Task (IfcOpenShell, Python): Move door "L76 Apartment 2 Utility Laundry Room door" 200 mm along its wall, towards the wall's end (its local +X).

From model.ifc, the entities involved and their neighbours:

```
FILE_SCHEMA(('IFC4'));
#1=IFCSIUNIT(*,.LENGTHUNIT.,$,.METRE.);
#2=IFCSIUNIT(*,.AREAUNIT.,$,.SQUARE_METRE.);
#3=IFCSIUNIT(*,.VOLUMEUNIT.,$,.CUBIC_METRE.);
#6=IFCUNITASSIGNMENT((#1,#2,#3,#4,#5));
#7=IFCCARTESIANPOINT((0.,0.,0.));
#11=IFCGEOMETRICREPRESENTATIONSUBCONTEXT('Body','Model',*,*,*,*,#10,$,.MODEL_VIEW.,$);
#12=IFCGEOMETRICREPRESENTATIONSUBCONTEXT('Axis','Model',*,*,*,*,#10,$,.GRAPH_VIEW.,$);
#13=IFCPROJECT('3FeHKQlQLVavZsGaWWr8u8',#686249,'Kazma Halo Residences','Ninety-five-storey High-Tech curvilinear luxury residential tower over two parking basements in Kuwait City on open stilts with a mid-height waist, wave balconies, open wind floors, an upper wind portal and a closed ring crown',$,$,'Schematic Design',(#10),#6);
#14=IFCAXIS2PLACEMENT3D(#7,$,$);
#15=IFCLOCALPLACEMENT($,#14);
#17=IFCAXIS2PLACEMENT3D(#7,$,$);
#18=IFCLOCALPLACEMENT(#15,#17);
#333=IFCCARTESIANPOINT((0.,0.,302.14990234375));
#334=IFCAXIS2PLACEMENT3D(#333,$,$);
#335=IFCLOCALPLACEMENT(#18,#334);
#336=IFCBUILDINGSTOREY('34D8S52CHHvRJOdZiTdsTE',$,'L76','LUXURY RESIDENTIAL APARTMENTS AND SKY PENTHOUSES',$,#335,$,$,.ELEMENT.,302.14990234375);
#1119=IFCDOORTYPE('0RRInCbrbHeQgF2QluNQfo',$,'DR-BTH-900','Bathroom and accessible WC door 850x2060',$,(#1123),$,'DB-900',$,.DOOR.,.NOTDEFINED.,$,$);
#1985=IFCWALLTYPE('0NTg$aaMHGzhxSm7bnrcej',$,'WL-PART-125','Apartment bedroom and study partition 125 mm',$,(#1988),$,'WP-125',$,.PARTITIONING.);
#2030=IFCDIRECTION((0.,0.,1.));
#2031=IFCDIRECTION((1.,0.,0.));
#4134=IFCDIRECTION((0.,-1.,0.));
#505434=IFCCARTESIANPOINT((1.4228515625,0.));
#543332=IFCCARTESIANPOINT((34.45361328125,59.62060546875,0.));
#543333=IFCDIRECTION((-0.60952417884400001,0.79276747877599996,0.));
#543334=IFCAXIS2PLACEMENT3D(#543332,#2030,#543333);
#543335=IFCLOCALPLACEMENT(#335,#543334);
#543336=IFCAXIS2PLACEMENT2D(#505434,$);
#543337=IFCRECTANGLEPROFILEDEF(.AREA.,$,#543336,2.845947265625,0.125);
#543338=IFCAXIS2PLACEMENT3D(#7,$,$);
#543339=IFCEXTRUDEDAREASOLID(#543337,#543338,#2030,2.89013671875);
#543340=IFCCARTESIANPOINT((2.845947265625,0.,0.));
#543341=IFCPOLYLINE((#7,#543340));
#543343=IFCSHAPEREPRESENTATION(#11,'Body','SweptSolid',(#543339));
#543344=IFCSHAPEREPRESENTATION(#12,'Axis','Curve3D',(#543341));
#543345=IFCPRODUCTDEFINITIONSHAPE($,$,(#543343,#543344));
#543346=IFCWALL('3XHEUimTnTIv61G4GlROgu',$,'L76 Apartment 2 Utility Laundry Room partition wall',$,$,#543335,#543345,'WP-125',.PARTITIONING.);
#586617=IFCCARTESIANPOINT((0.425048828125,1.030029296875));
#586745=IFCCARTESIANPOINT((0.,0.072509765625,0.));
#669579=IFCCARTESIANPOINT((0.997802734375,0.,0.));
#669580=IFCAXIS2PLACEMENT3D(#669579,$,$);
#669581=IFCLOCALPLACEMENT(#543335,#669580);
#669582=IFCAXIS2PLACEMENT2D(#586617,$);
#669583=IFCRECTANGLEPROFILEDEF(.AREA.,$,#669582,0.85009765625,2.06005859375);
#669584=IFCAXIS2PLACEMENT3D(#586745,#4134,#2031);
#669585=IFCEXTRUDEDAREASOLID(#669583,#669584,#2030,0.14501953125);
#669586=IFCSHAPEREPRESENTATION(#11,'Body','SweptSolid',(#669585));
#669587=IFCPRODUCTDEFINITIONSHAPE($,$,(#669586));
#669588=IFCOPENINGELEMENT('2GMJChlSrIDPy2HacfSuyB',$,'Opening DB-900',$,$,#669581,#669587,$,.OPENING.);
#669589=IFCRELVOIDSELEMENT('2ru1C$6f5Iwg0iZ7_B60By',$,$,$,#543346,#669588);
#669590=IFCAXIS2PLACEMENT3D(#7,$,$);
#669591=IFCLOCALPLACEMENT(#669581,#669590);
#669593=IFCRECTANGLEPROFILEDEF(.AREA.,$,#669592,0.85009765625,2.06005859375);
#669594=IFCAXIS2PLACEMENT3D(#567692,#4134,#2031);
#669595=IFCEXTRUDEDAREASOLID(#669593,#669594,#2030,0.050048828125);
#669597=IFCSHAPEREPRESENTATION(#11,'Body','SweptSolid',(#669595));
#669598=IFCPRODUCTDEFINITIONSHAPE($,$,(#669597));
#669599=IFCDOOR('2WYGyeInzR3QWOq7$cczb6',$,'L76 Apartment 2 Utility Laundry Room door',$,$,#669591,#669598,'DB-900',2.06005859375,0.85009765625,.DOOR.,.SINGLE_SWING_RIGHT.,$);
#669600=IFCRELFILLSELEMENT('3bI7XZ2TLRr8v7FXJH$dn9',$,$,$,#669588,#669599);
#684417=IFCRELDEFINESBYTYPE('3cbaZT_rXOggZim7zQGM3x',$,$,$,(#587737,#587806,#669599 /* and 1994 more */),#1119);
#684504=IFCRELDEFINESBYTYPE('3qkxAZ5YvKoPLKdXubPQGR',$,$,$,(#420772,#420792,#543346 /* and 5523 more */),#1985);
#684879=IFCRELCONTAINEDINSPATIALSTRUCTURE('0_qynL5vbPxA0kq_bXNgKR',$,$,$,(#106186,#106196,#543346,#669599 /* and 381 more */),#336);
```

```python
import ifcopenshell
import ifcopenshell.api.geometry
import ifcopenshell.util.placement

model = ifcopenshell.open("model.ifc")

door = model.by_id(669599)
opening = door.FillsVoids[0].RelatingOpeningElement
wall = opening.VoidsElements[0].RelatingBuildingElement

wall_matrix = ifcopenshell.util.placement.get_local_placement(wall.ObjectPlacement)
shift = wall_matrix[:3, 0] * 0.2
before = ifcopenshell.util.placement.get_local_placement(door.ObjectPlacement)[:3, 3].copy()

# The door is placed relative to its opening, so it follows when the opening moves.
matrix = ifcopenshell.util.placement.get_local_placement(opening.ObjectPlacement)
matrix[:3, 3] += shift
ifcopenshell.api.geometry.edit_object_placement(
    model, product=opening, matrix=matrix, is_si=False, should_transform_children=True
)

after = ifcopenshell.util.placement.get_local_placement(door.ObjectPlacement)[:3, 3]
print("door moved by", (after - before).round(3) + 0.0)

model.write("model_v2.ifc")
```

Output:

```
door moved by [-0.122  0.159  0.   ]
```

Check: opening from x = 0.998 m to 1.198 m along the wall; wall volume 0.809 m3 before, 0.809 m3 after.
